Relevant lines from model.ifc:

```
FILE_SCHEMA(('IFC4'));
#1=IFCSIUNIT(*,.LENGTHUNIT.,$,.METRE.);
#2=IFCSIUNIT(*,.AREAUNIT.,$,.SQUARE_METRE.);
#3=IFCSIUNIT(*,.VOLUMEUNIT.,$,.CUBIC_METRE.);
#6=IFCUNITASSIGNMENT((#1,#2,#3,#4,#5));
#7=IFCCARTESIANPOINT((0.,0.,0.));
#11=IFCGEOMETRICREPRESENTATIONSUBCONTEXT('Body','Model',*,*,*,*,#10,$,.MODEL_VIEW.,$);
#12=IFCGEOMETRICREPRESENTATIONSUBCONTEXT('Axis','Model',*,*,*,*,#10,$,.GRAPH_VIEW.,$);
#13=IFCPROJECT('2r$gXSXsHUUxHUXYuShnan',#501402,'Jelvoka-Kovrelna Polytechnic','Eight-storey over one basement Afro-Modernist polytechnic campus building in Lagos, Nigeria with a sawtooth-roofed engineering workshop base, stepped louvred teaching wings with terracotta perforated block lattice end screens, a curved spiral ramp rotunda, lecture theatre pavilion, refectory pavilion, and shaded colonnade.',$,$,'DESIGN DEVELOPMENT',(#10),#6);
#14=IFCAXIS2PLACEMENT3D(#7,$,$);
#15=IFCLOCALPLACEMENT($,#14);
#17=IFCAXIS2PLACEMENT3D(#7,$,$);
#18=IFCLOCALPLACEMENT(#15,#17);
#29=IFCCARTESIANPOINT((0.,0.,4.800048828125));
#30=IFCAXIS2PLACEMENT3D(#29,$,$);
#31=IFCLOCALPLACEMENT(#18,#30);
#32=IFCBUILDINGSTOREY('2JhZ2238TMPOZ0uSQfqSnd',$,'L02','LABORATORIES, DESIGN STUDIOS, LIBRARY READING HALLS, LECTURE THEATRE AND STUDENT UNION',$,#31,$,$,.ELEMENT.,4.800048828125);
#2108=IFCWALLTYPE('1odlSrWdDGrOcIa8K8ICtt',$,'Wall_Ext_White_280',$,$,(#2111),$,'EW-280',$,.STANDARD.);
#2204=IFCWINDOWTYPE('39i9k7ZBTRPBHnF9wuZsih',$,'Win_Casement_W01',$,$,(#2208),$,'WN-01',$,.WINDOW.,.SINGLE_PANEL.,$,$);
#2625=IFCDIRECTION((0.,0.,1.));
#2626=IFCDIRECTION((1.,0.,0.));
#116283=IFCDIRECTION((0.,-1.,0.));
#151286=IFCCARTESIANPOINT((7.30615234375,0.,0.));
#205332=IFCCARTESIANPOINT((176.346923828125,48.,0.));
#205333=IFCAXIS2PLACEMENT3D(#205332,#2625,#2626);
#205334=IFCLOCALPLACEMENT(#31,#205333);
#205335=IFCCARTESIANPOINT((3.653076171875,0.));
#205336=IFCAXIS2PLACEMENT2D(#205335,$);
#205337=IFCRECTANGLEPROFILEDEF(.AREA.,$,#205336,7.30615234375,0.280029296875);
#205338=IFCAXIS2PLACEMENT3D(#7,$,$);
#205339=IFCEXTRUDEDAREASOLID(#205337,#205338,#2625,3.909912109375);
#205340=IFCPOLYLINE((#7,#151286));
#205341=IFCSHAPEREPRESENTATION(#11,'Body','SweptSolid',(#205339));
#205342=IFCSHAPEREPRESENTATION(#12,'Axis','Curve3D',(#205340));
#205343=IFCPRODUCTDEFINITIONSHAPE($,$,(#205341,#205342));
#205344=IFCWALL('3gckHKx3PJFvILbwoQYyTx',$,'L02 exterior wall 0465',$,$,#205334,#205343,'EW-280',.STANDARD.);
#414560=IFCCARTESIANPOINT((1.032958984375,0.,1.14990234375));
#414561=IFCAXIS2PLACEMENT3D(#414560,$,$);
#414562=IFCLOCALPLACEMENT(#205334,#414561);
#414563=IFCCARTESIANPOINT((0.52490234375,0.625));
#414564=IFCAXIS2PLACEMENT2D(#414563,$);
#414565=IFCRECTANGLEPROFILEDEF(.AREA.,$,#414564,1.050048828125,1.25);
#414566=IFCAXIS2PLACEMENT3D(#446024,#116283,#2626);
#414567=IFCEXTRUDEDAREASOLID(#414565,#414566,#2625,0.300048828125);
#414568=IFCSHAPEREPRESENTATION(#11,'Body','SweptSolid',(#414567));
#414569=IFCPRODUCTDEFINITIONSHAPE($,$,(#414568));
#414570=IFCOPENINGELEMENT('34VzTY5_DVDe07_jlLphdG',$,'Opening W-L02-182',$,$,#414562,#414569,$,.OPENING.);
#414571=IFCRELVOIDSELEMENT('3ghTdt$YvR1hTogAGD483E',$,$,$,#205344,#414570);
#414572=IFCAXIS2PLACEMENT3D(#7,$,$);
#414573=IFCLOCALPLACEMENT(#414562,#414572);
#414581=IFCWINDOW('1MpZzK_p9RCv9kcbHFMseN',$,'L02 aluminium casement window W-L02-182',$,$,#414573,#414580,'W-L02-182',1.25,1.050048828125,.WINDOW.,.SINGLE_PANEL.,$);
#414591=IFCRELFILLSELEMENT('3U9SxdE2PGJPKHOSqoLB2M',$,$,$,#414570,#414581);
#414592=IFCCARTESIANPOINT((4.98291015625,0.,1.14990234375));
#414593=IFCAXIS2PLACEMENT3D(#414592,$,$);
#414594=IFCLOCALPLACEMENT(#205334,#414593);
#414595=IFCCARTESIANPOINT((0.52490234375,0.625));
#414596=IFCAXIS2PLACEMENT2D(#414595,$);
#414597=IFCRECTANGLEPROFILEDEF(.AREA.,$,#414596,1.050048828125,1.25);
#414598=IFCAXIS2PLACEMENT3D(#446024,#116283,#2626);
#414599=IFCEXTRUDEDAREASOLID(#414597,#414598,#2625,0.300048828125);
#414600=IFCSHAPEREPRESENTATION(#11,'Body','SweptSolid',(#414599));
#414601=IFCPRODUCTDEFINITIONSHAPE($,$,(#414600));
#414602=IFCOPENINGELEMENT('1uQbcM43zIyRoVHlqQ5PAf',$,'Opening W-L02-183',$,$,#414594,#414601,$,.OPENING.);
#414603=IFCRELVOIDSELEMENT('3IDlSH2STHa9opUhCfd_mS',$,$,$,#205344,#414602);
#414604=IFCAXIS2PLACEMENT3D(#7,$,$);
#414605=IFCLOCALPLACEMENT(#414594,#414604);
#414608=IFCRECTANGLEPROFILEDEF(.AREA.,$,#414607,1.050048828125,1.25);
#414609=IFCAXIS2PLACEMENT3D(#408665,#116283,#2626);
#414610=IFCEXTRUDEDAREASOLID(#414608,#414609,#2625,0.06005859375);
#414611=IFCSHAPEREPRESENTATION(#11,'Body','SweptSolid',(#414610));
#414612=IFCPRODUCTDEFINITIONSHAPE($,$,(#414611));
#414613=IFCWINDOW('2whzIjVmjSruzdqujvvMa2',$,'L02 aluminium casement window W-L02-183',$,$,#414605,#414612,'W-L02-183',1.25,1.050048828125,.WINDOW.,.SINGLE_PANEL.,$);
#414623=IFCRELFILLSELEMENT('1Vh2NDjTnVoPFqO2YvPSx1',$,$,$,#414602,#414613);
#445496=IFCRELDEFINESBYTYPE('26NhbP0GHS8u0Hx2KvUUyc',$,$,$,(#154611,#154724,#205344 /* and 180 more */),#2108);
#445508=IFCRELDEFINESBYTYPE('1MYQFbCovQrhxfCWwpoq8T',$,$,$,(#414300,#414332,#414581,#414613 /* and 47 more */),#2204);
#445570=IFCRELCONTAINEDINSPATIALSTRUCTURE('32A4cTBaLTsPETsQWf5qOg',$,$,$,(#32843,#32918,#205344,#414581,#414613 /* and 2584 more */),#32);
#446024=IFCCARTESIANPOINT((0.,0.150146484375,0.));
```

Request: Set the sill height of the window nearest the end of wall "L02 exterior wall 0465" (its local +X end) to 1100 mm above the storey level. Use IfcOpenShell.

```python
import numpy as np
import ifcopenshell
import ifcopenshell.api.geometry
import ifcopenshell.geom
import ifcopenshell.util.element
import ifcopenshell.util.placement
import ifcopenshell.util.shape
import ifcopenshell.util.unit

model = ifcopenshell.open("model.ifc")
unit_scale = ifcopenshell.util.unit.calculate_unit_scale(model)

window = model.by_guid("2whzIjVmjSruzdqujvvMa2")
opening = window.FillsVoids[0].RelatingOpeningElement
storey = ifcopenshell.util.element.get_container(window, ifc_class="IfcBuildingStorey")
level = ifcopenshell.util.placement.get_local_placement(storey.ObjectPlacement)[2, 3]

# The opening's origin need not be at the sill, so measure its lowest point.
shape = ifcopenshell.geom.create_shape(ifcopenshell.geom.settings(), opening)
bottom = ifcopenshell.util.shape.get_shape_bottom_elevation(shape, shape.geometry) / unit_scale
dz = level + 1.1 / unit_scale - bottom

shift = np.array([0.0, 0.0, dz])
# The window is placed relative to its opening, so it follows when the opening moves.
matrix = ifcopenshell.util.placement.get_local_placement(opening.ObjectPlacement)
matrix[:3, 3] += shift
ifcopenshell.api.geometry.edit_object_placement(
    model, product=opening, matrix=matrix, is_si=False, should_transform_children=True
)

print(f"moved by {dz * unit_scale:+.3f} m")

model.write("model_updated.ifc")
```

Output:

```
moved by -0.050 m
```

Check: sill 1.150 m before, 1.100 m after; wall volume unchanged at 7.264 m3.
